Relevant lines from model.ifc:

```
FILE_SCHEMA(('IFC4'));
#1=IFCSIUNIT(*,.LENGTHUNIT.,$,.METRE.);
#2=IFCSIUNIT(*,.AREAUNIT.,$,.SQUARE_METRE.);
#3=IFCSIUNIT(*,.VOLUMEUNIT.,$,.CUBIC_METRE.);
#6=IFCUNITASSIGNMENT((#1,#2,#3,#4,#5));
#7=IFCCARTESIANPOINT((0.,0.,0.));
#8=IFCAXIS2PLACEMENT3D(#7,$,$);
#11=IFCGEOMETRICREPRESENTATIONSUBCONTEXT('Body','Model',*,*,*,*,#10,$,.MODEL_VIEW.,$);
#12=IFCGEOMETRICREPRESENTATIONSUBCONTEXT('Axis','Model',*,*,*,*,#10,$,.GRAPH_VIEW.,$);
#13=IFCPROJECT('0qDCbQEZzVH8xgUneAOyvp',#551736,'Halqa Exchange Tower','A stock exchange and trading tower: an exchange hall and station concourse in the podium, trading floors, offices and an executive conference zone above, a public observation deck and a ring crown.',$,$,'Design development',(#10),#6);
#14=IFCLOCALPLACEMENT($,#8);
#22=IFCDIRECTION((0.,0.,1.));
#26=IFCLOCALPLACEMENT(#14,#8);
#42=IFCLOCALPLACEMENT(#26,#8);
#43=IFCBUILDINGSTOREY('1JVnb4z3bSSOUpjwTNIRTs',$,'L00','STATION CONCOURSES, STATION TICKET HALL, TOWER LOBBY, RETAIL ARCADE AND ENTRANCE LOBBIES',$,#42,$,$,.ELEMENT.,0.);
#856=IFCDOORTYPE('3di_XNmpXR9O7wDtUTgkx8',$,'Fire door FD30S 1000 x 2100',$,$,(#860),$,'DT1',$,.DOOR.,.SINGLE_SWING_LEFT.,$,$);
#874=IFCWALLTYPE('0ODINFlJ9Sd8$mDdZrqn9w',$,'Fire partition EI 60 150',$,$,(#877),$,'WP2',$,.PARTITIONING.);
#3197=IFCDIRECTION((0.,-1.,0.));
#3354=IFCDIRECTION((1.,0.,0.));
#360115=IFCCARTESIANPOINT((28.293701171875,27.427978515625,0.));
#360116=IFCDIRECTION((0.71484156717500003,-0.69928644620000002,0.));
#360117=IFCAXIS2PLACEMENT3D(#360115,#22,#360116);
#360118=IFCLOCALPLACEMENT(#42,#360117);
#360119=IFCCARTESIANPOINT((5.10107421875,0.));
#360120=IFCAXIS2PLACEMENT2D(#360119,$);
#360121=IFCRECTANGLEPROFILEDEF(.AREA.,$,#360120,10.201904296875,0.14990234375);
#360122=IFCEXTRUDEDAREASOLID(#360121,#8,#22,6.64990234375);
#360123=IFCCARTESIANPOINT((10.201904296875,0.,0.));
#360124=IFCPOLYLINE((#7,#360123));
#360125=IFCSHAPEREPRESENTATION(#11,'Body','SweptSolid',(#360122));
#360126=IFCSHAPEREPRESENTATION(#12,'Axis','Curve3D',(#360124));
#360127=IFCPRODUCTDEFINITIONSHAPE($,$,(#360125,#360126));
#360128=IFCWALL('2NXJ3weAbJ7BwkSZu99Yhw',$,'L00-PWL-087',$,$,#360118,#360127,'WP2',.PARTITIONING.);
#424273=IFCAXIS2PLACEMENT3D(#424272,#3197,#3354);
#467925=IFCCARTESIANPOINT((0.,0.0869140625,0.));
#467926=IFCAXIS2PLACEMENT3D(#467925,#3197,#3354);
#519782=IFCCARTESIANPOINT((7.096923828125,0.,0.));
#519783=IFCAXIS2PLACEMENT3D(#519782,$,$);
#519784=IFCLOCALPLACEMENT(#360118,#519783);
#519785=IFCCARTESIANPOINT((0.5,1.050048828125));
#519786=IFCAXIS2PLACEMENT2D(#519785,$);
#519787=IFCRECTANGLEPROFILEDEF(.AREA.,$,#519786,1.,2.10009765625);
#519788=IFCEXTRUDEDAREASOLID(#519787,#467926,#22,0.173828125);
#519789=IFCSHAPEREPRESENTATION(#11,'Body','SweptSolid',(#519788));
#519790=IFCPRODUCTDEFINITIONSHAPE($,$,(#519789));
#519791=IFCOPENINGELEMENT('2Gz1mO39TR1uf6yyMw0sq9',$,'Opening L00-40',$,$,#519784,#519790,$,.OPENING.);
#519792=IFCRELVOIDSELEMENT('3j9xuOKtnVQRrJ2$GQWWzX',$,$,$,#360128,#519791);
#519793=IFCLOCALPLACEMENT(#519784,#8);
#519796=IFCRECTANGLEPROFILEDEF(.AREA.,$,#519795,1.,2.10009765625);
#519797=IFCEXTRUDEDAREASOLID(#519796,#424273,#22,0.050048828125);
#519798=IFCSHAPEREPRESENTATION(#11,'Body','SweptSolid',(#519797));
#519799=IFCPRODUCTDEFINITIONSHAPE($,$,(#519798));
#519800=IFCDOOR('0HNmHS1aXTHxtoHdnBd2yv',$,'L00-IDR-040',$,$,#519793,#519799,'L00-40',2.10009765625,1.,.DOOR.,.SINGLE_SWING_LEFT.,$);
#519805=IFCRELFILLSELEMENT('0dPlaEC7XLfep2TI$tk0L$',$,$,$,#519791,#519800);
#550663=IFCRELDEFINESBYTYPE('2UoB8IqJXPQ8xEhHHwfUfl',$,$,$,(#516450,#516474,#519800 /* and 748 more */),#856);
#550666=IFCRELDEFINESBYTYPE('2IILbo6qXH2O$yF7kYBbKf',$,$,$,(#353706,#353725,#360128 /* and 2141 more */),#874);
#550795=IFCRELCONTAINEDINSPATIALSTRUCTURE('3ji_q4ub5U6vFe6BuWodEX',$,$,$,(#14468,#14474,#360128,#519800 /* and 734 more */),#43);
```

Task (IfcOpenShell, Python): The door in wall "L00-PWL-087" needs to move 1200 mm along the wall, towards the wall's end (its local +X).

```python
import ifcopenshell
import ifcopenshell.api.geometry
import ifcopenshell.util.placement
import ifcopenshell.util.unit

model = ifcopenshell.open("model.ifc")
unit_scale = ifcopenshell.util.unit.calculate_unit_scale(model)

door = model.by_id(519800)
opening = door.FillsVoids[0].RelatingOpeningElement
wall = opening.VoidsElements[0].RelatingBuildingElement

wall_matrix = ifcopenshell.util.placement.get_local_placement(wall.ObjectPlacement)
shift = wall_matrix[:3, 0] * 1.2 / unit_scale
before = ifcopenshell.util.placement.get_local_placement(door.ObjectPlacement)[:3, 3].copy()

# The door is placed relative to its opening, so it follows when the opening moves.
matrix = ifcopenshell.util.placement.get_local_placement(opening.ObjectPlacement)
matrix[:3, 3] += shift
ifcopenshell.api.geometry.edit_object_placement(
    model, product=opening, matrix=matrix, is_si=False, should_transform_children=True
)

after = ifcopenshell.util.placement.get_local_placement(door.ObjectPlacement)[:3, 3]
print("door moved by", (after - before).round(3) + 0.0)

model.write("model_v2.ifc")
```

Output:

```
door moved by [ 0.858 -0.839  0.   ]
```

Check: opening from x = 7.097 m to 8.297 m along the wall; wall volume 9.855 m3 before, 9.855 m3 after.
